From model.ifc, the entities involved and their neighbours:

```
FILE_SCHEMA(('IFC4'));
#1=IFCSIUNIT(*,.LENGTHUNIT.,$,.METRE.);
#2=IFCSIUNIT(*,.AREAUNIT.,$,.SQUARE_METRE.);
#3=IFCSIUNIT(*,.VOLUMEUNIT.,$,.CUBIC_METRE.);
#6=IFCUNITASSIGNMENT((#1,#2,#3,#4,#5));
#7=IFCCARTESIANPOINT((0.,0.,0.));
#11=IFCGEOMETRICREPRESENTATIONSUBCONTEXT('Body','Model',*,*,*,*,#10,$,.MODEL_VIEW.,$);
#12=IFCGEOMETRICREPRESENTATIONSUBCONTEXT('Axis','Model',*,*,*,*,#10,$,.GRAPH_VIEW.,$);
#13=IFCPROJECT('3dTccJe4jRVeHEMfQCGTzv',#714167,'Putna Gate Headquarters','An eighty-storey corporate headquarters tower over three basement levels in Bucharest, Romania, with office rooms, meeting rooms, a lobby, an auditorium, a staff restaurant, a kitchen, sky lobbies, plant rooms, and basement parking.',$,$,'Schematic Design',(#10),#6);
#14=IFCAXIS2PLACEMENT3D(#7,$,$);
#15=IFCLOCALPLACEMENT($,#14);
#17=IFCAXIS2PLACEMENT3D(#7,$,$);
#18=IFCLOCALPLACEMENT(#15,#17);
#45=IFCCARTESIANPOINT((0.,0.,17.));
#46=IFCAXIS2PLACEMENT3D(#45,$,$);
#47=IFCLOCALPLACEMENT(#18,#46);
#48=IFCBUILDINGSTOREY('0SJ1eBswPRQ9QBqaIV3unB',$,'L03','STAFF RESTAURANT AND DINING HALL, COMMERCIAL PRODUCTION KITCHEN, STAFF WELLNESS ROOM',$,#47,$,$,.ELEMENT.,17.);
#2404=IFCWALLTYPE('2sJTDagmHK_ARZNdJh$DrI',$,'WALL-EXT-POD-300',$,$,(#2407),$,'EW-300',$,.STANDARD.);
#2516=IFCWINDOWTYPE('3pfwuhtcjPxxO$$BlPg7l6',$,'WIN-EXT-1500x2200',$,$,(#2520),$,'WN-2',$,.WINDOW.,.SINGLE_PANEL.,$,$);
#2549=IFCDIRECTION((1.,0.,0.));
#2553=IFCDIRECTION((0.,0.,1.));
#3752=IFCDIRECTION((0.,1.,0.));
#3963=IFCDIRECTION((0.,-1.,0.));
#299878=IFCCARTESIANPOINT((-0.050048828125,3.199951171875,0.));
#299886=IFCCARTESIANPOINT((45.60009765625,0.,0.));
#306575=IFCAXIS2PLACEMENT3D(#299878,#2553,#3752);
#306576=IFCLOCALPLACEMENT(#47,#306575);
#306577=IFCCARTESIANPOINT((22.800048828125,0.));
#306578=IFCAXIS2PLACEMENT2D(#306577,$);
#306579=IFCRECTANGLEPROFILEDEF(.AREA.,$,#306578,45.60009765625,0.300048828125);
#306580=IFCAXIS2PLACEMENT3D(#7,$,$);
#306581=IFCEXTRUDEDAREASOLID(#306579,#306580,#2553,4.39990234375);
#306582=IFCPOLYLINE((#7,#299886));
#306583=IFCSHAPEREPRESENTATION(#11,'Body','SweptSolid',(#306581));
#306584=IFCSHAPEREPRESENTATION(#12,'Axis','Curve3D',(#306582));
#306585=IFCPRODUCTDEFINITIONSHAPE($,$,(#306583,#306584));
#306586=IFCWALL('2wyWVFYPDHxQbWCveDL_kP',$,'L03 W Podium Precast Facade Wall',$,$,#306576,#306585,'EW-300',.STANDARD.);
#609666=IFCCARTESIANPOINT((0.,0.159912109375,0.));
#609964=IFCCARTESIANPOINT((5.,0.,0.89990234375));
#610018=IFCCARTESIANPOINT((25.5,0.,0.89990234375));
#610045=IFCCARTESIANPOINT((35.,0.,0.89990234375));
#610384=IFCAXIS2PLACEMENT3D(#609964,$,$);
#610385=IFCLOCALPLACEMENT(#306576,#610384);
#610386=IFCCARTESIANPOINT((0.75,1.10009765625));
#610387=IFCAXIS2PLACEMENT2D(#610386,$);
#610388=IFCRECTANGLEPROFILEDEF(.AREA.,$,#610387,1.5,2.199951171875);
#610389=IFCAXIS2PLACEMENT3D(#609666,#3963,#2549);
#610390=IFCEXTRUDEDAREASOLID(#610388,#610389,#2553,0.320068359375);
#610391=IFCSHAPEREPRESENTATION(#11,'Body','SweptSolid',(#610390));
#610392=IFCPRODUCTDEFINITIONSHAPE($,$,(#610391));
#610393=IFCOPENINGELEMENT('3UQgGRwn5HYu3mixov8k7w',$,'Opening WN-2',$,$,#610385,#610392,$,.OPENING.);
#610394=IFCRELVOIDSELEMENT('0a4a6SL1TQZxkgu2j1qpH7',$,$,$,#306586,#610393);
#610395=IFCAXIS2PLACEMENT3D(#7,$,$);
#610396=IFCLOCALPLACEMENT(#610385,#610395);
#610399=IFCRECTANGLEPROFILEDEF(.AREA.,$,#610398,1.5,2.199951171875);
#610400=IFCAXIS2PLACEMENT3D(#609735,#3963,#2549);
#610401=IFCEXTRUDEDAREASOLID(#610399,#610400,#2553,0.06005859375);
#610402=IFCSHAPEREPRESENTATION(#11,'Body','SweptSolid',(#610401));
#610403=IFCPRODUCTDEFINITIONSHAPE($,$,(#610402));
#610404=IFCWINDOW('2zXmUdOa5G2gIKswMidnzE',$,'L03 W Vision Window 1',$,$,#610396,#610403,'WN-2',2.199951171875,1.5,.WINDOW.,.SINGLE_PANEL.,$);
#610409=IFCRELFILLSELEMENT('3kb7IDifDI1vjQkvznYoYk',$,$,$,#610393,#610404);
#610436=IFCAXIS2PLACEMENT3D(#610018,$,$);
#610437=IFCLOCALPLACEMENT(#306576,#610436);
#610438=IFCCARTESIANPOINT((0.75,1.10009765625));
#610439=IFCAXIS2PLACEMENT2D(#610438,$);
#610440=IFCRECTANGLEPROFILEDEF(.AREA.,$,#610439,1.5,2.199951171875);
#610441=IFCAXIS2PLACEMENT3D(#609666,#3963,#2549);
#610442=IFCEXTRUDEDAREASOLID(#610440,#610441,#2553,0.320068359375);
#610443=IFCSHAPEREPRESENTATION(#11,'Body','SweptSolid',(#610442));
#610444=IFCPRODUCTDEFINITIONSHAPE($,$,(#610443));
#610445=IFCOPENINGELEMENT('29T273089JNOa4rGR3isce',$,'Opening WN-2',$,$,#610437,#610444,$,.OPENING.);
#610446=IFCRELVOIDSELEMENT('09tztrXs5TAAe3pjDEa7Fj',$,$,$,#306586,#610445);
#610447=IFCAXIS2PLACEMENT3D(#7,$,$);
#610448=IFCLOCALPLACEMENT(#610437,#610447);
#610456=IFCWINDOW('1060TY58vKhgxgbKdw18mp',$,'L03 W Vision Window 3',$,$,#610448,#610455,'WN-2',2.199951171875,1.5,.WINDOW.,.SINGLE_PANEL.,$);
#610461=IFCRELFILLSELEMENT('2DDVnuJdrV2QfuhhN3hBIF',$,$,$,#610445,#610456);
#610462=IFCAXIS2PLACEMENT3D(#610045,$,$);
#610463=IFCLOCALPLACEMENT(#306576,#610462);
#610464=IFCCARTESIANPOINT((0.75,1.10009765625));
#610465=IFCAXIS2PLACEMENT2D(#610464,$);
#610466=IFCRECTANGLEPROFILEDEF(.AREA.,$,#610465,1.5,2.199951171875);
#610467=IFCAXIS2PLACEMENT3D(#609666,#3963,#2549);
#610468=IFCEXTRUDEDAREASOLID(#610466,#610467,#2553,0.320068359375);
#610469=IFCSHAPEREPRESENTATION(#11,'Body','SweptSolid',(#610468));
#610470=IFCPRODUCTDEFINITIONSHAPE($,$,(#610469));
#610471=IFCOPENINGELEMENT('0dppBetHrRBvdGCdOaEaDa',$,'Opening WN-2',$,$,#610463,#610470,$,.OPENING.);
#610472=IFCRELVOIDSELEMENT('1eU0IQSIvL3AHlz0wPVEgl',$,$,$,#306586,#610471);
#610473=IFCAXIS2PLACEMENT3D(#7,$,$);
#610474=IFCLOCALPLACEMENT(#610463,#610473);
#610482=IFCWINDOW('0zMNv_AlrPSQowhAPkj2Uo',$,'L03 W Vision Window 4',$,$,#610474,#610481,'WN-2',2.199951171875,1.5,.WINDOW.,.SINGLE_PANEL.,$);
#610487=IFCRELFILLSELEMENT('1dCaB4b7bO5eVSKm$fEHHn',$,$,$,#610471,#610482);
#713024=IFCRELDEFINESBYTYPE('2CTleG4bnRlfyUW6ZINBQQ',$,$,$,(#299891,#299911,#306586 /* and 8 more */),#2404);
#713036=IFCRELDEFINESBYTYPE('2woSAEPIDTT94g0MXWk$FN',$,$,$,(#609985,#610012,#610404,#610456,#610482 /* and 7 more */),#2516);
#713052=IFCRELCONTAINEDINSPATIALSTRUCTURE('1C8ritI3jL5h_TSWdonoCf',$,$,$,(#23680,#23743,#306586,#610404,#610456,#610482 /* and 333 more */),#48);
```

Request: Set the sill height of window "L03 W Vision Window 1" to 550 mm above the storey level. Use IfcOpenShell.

```python
import numpy as np
import ifcopenshell
import ifcopenshell.api.geometry
import ifcopenshell.geom
import ifcopenshell.util.element
import ifcopenshell.util.placement
import ifcopenshell.util.shape
import ifcopenshell.util.unit

model = ifcopenshell.open("model.ifc")
unit_scale = ifcopenshell.util.unit.calculate_unit_scale(model)

window = model.by_guid("2zXmUdOa5G2gIKswMidnzE")
opening = window.FillsVoids[0].RelatingOpeningElement
storey = ifcopenshell.util.element.get_container(window, ifc_class="IfcBuildingStorey")
level = ifcopenshell.util.placement.get_local_placement(storey.ObjectPlacement)[2, 3]

# The opening's origin need not be at the sill, so measure its lowest point.
shape = ifcopenshell.geom.create_shape(ifcopenshell.geom.settings(), opening)
bottom = ifcopenshell.util.shape.get_shape_bottom_elevation(shape, shape.geometry) / unit_scale
dz = level + 0.55 / unit_scale - bottom

shift = np.array([0.0, 0.0, dz])
# The window is placed relative to its opening, so it follows when the opening moves.
matrix = ifcopenshell.util.placement.get_local_placement(opening.ObjectPlacement)
matrix[:3, 3] += shift
ifcopenshell.api.geometry.edit_object_placement(
    model, product=opening, matrix=matrix, is_si=False, should_transform_children=True
)

print(f"moved by {dz * unit_scale:+.3f} m")

model.write("model_edited.ifc")
```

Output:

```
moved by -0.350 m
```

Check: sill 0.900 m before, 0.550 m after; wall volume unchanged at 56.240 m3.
